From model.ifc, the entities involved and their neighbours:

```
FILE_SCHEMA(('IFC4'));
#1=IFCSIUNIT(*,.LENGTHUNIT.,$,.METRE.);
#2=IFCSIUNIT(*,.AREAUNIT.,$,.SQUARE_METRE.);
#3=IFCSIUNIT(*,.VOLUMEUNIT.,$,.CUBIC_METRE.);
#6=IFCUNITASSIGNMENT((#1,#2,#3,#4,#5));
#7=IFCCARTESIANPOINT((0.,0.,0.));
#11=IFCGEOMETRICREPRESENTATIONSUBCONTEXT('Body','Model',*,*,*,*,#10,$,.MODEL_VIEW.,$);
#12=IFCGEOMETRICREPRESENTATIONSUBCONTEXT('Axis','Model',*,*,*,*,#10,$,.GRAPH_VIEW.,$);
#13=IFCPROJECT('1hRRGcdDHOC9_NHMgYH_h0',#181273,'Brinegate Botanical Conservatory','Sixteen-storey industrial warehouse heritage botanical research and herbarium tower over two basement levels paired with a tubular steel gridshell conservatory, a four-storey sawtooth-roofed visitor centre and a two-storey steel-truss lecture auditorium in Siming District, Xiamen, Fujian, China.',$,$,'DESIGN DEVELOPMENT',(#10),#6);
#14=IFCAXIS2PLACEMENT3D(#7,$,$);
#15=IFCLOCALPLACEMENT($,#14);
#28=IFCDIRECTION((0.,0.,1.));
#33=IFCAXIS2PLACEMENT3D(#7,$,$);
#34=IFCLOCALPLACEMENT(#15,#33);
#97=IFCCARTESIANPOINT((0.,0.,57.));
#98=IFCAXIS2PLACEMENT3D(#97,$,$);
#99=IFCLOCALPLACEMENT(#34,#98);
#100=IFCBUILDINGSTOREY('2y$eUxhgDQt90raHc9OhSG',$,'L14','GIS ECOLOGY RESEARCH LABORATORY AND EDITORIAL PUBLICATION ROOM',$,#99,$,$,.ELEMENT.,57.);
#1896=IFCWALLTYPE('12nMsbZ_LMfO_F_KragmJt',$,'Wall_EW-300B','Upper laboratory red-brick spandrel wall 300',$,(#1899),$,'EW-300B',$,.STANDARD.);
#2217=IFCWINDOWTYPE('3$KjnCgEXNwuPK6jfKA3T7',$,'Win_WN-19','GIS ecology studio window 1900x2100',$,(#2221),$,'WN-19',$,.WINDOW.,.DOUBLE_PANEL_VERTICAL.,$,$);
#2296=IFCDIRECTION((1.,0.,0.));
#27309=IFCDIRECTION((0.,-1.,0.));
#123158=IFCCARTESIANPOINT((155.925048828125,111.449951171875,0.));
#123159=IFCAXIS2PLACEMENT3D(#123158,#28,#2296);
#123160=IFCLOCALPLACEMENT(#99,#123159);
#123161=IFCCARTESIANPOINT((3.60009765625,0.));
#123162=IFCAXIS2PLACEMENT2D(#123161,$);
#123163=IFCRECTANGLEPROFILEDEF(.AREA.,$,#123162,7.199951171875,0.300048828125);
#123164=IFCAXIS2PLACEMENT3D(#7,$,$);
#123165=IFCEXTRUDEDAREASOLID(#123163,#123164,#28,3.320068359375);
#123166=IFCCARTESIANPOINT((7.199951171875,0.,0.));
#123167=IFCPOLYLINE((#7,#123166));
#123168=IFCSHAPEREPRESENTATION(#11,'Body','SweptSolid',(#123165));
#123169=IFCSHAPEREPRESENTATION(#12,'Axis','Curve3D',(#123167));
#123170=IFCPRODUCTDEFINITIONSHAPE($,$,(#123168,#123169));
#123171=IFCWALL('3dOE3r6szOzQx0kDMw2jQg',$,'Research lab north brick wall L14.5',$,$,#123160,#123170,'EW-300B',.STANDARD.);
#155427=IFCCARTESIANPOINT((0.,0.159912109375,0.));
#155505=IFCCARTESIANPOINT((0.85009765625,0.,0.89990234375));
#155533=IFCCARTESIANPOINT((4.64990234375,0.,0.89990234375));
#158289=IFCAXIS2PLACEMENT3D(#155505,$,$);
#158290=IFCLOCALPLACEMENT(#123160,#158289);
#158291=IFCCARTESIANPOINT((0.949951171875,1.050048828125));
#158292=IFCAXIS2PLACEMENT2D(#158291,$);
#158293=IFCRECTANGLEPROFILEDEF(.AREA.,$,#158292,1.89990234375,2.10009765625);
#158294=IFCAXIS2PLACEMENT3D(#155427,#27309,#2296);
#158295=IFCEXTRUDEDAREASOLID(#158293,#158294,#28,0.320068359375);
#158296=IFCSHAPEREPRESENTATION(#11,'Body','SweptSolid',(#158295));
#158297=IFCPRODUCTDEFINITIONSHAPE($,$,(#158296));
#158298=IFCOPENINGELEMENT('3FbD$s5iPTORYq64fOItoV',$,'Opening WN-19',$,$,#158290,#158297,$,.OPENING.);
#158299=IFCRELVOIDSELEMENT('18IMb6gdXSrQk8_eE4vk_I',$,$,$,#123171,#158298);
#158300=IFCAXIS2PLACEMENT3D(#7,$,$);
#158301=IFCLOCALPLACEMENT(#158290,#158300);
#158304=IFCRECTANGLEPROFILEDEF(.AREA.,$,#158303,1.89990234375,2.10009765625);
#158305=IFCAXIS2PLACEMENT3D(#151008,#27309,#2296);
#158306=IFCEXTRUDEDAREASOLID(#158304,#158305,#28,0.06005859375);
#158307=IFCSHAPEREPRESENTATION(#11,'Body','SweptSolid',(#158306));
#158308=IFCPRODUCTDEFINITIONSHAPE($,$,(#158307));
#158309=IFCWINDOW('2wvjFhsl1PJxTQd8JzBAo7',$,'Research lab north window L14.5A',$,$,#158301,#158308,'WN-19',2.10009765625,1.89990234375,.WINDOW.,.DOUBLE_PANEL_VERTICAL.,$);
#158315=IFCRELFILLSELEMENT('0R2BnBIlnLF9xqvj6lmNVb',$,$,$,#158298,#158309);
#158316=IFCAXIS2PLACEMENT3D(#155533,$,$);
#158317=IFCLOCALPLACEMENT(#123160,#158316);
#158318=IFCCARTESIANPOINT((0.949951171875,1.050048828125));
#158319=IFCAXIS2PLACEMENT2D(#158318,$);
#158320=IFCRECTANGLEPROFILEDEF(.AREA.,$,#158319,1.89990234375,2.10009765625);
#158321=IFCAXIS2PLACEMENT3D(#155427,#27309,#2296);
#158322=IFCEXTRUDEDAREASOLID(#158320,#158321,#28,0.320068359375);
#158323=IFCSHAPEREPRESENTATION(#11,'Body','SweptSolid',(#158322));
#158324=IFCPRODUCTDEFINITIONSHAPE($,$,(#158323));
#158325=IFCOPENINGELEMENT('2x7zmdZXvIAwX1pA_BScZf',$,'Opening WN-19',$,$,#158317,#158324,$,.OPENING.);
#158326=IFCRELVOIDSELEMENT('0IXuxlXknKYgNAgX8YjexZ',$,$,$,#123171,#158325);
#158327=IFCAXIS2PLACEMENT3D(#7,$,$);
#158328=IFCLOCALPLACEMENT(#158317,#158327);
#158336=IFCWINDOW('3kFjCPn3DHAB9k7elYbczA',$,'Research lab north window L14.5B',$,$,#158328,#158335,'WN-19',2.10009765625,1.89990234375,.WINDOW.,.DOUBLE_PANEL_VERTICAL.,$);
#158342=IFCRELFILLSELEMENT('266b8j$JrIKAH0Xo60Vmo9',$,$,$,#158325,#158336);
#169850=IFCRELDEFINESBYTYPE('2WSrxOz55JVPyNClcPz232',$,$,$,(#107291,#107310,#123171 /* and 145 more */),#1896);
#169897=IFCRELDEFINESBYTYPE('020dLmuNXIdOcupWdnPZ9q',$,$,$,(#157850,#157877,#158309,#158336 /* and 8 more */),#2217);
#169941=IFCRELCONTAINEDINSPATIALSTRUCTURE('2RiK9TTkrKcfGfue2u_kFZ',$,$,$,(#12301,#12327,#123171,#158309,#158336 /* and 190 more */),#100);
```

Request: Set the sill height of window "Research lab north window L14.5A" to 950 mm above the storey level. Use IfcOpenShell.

```python
import numpy as np
import ifcopenshell
import ifcopenshell.api.geometry
import ifcopenshell.geom
import ifcopenshell.util.element
import ifcopenshell.util.placement
import ifcopenshell.util.shape
import ifcopenshell.util.unit

model = ifcopenshell.open("model.ifc")
unit_scale = ifcopenshell.util.unit.calculate_unit_scale(model)

window = model.by_guid("2wvjFhsl1PJxTQd8JzBAo7")
opening = window.FillsVoids[0].RelatingOpeningElement
storey = ifcopenshell.util.element.get_container(window, ifc_class="IfcBuildingStorey")
level = ifcopenshell.util.placement.get_local_placement(storey.ObjectPlacement)[2, 3]

# The opening's origin need not be at the sill, so measure its lowest point.
shape = ifcopenshell.geom.create_shape(ifcopenshell.geom.settings(), opening)
bottom = ifcopenshell.util.shape.get_shape_bottom_elevation(shape, shape.geometry) / unit_scale
dz = level + 0.95 / unit_scale - bottom

shift = np.array([0.0, 0.0, dz])
# The window is placed relative to its opening, so it follows when the opening moves.
matrix = ifcopenshell.util.placement.get_local_placement(opening.ObjectPlacement)
matrix[:3, 3] += shift
ifcopenshell.api.geometry.edit_object_placement(
    model, product=opening, matrix=matrix, is_si=False, should_transform_children=True
)

print(f"moved by {dz * unit_scale:+.3f} m")

model.write("model_v2.ifc")
```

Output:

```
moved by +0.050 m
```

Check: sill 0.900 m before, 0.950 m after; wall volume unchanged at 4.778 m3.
